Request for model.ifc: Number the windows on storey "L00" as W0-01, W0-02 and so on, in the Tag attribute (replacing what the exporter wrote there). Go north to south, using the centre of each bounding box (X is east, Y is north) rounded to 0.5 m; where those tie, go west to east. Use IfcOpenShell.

First a look at what the model holds.

```python
import ifcopenshell
import ifcopenshell.util.element
import ifcopenshell.util.placement

model = ifcopenshell.open("model.ifc")
print(model.schema)
storey = next(s for s in model.by_type("IfcBuildingStorey") if s.Name == "L00")
windows = [e for e in ifcopenshell.util.element.get_decomposition(storey) if e.is_a("IfcWindow")]
for e in sorted(windows, key=lambda e: e.id()):
    origin = ifcopenshell.util.placement.get_local_placement(e.ObjectPlacement)[:3, 3]
    print(e.id(), e.Tag, e.Name, origin.round(2) + 0.0, sep=" | ")
```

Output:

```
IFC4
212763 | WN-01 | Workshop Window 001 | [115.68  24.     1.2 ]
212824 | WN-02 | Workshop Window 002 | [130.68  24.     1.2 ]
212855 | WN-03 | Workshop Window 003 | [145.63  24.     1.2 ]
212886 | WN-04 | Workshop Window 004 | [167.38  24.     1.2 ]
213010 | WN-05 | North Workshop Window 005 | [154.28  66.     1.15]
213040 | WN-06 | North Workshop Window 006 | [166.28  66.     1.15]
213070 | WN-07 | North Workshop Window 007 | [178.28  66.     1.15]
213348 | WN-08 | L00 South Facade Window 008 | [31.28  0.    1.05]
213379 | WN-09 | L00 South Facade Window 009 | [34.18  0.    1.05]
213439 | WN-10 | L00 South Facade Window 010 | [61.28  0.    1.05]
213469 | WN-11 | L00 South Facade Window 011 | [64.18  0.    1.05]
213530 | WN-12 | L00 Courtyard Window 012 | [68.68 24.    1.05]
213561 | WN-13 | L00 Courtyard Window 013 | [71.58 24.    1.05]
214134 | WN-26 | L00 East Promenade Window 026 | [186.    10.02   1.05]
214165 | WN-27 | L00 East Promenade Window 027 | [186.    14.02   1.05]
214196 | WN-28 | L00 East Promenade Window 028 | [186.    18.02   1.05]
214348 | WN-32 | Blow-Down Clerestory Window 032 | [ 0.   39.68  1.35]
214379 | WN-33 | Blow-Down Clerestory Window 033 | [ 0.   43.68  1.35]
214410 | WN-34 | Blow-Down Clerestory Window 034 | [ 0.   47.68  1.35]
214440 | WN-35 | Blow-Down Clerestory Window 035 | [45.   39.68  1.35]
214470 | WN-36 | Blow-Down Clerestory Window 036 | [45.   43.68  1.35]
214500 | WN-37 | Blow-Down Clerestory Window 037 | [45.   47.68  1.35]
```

```python
import ifcopenshell
import ifcopenshell.geom
import ifcopenshell.util.element
import ifcopenshell.util.shape

model = ifcopenshell.open("model.ifc")
settings = ifcopenshell.geom.settings()
settings.set("use-world-coords", True)


def centre(element):
    shape = ifcopenshell.geom.create_shape(settings, element)
    return ifcopenshell.util.shape.get_bbox_centroid(shape.geometry)


storey = next(s for s in model.by_type("IfcBuildingStorey") if s.Name == "L00")
windows = [e for e in ifcopenshell.util.element.get_decomposition(storey) if e.is_a("IfcWindow")]

# Insertion points can sit at a corner or the storey origin, so sort by the geometry (in metres).
centres = {e: centre(e) for e in windows}
windows.sort(key=lambda e: (-round(centres[e][1] / 0.5), centres[e][0]))

for i, e in enumerate(windows, start=1):
    number = f"W0-{i:02d}"
    e.Tag = number
    print(e.id(), number)

model.write("model_rev.ifc")
```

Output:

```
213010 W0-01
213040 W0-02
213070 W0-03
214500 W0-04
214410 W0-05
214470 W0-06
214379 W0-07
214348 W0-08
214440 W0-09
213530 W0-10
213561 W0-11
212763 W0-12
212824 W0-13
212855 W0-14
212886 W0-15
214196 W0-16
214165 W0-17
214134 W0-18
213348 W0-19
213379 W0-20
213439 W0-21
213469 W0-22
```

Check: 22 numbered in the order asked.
